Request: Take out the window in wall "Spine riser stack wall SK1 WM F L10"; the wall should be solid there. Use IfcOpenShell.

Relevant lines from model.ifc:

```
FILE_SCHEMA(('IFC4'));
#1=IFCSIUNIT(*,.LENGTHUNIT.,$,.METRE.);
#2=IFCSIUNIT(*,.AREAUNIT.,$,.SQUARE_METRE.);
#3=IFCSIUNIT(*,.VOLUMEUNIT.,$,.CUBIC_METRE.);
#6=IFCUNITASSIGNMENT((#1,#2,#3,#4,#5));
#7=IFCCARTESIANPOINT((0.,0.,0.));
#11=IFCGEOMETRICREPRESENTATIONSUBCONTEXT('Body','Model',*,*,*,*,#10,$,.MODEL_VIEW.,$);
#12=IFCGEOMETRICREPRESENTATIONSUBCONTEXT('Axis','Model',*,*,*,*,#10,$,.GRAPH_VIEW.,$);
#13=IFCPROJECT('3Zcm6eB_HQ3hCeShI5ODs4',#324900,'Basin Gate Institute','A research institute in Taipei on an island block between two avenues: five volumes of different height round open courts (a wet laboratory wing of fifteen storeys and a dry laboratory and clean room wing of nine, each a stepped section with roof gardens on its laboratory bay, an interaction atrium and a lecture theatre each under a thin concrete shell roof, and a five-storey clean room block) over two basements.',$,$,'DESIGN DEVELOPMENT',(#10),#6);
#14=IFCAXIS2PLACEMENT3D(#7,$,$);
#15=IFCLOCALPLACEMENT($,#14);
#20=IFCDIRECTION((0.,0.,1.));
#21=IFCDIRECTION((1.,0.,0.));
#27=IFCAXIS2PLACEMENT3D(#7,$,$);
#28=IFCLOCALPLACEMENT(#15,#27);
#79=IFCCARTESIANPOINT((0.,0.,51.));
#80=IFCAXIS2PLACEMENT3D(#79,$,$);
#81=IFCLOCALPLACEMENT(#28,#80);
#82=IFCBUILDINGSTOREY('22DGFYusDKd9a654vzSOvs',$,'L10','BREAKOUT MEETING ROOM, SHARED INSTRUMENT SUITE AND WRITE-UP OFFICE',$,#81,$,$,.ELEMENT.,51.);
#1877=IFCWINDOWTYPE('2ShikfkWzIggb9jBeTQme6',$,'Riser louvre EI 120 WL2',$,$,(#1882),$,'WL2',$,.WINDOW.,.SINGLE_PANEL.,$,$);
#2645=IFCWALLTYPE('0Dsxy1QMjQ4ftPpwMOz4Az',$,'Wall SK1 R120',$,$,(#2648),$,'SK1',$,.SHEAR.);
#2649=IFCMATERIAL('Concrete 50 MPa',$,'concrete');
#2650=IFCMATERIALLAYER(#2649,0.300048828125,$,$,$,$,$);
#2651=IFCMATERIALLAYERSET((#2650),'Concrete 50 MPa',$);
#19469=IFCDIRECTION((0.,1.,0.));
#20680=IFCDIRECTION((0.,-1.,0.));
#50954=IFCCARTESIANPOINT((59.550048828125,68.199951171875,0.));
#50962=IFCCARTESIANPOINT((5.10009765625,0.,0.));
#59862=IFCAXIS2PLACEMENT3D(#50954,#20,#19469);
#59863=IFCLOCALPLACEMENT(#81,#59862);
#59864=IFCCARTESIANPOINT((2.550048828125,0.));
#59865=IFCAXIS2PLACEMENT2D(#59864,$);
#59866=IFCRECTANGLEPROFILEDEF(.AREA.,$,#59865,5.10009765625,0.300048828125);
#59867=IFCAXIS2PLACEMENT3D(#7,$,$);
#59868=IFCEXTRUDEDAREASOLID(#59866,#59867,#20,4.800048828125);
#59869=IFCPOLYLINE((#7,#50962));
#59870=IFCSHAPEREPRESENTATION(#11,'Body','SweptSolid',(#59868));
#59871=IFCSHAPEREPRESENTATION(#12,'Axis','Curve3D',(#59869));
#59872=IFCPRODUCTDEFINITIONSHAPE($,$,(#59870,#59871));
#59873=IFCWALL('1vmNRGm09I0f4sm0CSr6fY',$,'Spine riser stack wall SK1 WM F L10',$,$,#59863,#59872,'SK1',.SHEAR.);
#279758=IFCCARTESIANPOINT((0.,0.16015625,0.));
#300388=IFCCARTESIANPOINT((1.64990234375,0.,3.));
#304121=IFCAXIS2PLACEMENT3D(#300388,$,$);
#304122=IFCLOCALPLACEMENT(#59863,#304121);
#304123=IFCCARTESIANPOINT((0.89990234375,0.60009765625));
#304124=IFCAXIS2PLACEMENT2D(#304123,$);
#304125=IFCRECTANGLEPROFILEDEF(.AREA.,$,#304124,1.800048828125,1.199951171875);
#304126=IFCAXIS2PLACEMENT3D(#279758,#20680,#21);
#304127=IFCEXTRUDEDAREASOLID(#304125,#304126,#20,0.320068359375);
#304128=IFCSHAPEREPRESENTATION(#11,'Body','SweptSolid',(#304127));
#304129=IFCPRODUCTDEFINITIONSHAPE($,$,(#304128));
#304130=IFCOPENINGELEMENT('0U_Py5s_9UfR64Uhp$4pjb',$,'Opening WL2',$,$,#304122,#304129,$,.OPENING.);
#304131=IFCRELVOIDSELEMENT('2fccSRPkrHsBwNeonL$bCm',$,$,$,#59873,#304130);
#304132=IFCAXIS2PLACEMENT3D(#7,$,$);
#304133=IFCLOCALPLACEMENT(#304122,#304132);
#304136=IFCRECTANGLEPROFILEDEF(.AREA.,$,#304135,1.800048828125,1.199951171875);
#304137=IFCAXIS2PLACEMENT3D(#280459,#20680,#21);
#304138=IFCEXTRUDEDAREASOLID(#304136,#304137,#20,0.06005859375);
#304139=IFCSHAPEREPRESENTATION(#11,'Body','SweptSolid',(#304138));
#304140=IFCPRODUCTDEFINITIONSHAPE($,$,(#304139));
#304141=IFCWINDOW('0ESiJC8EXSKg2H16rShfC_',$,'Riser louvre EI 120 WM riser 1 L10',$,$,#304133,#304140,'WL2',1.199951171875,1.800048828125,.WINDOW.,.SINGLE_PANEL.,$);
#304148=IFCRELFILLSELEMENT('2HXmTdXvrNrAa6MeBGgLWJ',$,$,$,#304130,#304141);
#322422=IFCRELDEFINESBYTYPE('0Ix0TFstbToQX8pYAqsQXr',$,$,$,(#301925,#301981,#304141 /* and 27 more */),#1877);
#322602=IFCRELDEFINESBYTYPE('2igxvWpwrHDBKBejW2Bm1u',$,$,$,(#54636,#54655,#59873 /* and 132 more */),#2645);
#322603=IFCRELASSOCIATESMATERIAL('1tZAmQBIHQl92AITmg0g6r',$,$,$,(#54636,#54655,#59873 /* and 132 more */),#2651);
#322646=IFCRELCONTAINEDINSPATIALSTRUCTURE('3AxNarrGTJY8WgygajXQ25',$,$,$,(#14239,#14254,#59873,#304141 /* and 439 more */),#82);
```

```python
import ifcopenshell
import ifcopenshell.api.feature
import ifcopenshell.api.root
import ifcopenshell.geom
import ifcopenshell.util.shape

model = ifcopenshell.open("model.ifc")
settings = ifcopenshell.geom.settings()


def volume(element):
    """Net volume in cubic metres, openings subtracted."""
    shape = ifcopenshell.geom.create_shape(settings, element)
    return ifcopenshell.util.shape.get_volume(shape.geometry)


window = model.by_guid("0ESiJC8EXSKg2H16rShfC_")
opening = window.FillsVoids[0].RelatingOpeningElement
wall = opening.VoidsElements[0].RelatingBuildingElement
before = volume(wall)

ifcopenshell.api.root.remove_product(model, product=window)
ifcopenshell.api.feature.remove_feature(model, feature=opening)

after = volume(wall)

print(f"wall volume {before:.3f} -> {after:.3f} m3")

model.write("model_edited.ifc")
```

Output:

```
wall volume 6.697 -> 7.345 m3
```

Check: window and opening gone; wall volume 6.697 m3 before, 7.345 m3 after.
